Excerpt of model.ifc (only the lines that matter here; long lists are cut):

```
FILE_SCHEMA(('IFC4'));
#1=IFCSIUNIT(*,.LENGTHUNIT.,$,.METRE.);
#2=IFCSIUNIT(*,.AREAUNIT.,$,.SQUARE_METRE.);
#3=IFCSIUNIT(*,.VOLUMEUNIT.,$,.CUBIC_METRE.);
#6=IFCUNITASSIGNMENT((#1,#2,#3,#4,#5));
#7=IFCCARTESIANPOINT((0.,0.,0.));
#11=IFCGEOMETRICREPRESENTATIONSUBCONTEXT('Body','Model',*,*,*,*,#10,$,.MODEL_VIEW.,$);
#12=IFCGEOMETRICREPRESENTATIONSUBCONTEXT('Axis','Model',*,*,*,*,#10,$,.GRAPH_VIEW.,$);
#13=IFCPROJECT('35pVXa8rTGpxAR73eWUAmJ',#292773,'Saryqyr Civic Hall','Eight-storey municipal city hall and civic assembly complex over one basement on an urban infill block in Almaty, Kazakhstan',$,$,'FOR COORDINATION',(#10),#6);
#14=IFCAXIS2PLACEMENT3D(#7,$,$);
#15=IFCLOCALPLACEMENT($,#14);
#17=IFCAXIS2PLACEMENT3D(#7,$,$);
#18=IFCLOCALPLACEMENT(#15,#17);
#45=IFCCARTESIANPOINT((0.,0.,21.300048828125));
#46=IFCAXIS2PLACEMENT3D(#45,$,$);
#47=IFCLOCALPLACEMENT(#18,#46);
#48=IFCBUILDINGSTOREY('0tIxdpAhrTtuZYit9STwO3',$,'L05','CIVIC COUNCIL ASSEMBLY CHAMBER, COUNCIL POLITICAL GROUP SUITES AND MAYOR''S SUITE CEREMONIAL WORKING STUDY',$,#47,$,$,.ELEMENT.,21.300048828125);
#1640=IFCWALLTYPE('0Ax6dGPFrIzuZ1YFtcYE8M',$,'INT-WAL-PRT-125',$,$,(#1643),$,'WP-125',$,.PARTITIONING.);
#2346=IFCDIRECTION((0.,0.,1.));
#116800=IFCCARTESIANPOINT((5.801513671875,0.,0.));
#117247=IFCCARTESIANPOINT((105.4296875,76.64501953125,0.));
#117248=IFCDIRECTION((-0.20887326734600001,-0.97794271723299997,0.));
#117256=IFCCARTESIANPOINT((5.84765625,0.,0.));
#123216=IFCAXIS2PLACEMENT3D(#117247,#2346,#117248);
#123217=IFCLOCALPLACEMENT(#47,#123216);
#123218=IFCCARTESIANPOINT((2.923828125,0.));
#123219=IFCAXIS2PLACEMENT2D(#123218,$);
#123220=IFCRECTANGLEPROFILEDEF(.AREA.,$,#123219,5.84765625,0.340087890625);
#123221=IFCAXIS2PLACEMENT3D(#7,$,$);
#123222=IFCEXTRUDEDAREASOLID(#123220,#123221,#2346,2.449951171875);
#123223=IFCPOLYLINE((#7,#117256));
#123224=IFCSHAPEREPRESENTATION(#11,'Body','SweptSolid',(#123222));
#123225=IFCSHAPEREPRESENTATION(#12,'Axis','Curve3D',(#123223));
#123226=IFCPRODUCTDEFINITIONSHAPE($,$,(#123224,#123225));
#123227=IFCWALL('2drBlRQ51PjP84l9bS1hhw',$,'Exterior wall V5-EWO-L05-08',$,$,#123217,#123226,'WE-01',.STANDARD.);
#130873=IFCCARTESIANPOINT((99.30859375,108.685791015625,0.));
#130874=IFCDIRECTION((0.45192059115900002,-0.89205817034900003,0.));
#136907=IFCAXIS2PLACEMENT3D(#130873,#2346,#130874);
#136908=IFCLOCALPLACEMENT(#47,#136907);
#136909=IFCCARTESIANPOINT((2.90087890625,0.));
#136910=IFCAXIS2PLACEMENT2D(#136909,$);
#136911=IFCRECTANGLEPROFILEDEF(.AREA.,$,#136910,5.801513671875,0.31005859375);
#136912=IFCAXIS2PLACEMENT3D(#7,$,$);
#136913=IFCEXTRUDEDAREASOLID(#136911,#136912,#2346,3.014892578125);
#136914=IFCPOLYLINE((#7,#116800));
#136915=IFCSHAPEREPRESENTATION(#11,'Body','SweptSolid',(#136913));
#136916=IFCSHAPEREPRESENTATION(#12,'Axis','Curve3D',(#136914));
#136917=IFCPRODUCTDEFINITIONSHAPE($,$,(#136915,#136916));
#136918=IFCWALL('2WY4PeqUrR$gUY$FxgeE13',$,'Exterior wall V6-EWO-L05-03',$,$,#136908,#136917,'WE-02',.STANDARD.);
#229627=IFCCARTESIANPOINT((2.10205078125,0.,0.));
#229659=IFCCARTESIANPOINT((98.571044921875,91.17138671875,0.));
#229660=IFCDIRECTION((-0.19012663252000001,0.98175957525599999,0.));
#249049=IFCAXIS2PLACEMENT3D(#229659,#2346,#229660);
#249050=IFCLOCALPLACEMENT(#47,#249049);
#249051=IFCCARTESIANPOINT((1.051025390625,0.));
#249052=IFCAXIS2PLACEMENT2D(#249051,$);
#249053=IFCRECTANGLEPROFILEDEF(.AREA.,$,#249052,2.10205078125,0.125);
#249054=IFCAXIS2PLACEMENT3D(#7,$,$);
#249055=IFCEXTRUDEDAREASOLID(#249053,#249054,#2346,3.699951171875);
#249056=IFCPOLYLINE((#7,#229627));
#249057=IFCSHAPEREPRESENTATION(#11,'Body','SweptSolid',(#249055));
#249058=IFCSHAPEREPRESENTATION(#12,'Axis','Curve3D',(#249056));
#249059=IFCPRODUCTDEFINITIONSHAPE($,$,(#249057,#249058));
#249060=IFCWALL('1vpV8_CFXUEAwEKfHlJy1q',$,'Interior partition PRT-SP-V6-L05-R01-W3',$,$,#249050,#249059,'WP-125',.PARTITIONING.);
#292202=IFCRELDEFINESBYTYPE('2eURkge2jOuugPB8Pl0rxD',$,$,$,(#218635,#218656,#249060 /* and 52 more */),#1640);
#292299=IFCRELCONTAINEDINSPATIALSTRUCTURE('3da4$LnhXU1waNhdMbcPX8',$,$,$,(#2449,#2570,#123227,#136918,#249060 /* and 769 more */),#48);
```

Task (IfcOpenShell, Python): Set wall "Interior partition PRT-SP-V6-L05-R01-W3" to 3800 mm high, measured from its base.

```python
import ifcopenshell
import ifcopenshell.geom
import ifcopenshell.util.representation
import ifcopenshell.util.shape
import ifcopenshell.util.unit

model = ifcopenshell.open("model.ifc")
unit_scale = ifcopenshell.util.unit.calculate_unit_scale(model)
settings = ifcopenshell.geom.settings()


def volume(element):
    """Net volume in cubic metres, openings subtracted."""
    shape = ifcopenshell.geom.create_shape(settings, element)
    return ifcopenshell.util.shape.get_volume(shape.geometry)


wall = model.by_guid("1vpV8_CFXUEAwEKfHlJy1q")
before = volume(wall)

body = ifcopenshell.util.representation.get_representation(wall, "Model", "Body")
solid = body.Items[0]
old_height = solid.Depth
solid.Depth = 3.8 / unit_scale
after = volume(wall)

print(f"height {old_height:g} -> {solid.Depth:g}, volume {before:.3f} -> {after:.3f} m3")

model.write("model_updated.ifc")
```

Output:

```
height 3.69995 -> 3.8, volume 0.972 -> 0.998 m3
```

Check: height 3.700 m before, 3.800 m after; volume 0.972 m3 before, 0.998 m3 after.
